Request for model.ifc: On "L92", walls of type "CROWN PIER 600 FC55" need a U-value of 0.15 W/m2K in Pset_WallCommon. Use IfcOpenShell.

First a look at what the model holds.

```python
import ifcopenshell
import ifcopenshell.util.element

model = ifcopenshell.open("model.ifc")
print(model.schema)
storey = next(s for s in model.by_type("IfcBuildingStorey") if s.Name == "L92")
walls = [e for e in ifcopenshell.util.element.get_decomposition(storey) if e.is_a("IfcWall")]
seen = {}
for e in walls:
    element_type = ifcopenshell.util.element.get_type(e)
    key = (element_type.Name if element_type != e and element_type else None, ifcopenshell.util.element.get_pset(e, "Pset_WallCommon", "ThermalTransmittance"))
    seen[key] = seen.get(key, 0) + 1
for (name, value), count in sorted(seen.items(), key=str):
    print(count, "x", name, "|", value)
```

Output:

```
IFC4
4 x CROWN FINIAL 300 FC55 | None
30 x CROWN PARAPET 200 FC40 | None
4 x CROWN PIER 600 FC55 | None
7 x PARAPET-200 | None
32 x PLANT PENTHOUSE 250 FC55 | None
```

```python
import ifcopenshell
import ifcopenshell.api.pset
import ifcopenshell.util.element

model = ifcopenshell.open("model.ifc")

storey = next(s for s in model.by_type("IfcBuildingStorey") if s.Name == "L92")
walls = [e for e in ifcopenshell.util.element.get_decomposition(storey) if e.is_a("IfcWall")]

count = 0
for e in walls:
    element_type = ifcopenshell.util.element.get_type(e)
    if element_type in (None, e) or element_type.Name != "CROWN PIER 600 FC55":
        continue
    found = ifcopenshell.util.element.get_pset(e, "Pset_WallCommon", should_inherit=False)
    if found:
        pset = model.by_id(found["id"])
        if len(ifcopenshell.util.element.get_elements_by_pset(pset)) > 1:
            pset = ifcopenshell.api.pset.unshare_pset(model, products=[e], pset=pset)[0]
    else:
        pset = ifcopenshell.api.pset.add_pset(model, product=e, name="Pset_WallCommon")
    ifcopenshell.api.pset.edit_pset(model, pset=pset, properties={"ThermalTransmittance": 0.15})
    count += 1

print(count, "walls updated")

model.write("model-out.ifc")
```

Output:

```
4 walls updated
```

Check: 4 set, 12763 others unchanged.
